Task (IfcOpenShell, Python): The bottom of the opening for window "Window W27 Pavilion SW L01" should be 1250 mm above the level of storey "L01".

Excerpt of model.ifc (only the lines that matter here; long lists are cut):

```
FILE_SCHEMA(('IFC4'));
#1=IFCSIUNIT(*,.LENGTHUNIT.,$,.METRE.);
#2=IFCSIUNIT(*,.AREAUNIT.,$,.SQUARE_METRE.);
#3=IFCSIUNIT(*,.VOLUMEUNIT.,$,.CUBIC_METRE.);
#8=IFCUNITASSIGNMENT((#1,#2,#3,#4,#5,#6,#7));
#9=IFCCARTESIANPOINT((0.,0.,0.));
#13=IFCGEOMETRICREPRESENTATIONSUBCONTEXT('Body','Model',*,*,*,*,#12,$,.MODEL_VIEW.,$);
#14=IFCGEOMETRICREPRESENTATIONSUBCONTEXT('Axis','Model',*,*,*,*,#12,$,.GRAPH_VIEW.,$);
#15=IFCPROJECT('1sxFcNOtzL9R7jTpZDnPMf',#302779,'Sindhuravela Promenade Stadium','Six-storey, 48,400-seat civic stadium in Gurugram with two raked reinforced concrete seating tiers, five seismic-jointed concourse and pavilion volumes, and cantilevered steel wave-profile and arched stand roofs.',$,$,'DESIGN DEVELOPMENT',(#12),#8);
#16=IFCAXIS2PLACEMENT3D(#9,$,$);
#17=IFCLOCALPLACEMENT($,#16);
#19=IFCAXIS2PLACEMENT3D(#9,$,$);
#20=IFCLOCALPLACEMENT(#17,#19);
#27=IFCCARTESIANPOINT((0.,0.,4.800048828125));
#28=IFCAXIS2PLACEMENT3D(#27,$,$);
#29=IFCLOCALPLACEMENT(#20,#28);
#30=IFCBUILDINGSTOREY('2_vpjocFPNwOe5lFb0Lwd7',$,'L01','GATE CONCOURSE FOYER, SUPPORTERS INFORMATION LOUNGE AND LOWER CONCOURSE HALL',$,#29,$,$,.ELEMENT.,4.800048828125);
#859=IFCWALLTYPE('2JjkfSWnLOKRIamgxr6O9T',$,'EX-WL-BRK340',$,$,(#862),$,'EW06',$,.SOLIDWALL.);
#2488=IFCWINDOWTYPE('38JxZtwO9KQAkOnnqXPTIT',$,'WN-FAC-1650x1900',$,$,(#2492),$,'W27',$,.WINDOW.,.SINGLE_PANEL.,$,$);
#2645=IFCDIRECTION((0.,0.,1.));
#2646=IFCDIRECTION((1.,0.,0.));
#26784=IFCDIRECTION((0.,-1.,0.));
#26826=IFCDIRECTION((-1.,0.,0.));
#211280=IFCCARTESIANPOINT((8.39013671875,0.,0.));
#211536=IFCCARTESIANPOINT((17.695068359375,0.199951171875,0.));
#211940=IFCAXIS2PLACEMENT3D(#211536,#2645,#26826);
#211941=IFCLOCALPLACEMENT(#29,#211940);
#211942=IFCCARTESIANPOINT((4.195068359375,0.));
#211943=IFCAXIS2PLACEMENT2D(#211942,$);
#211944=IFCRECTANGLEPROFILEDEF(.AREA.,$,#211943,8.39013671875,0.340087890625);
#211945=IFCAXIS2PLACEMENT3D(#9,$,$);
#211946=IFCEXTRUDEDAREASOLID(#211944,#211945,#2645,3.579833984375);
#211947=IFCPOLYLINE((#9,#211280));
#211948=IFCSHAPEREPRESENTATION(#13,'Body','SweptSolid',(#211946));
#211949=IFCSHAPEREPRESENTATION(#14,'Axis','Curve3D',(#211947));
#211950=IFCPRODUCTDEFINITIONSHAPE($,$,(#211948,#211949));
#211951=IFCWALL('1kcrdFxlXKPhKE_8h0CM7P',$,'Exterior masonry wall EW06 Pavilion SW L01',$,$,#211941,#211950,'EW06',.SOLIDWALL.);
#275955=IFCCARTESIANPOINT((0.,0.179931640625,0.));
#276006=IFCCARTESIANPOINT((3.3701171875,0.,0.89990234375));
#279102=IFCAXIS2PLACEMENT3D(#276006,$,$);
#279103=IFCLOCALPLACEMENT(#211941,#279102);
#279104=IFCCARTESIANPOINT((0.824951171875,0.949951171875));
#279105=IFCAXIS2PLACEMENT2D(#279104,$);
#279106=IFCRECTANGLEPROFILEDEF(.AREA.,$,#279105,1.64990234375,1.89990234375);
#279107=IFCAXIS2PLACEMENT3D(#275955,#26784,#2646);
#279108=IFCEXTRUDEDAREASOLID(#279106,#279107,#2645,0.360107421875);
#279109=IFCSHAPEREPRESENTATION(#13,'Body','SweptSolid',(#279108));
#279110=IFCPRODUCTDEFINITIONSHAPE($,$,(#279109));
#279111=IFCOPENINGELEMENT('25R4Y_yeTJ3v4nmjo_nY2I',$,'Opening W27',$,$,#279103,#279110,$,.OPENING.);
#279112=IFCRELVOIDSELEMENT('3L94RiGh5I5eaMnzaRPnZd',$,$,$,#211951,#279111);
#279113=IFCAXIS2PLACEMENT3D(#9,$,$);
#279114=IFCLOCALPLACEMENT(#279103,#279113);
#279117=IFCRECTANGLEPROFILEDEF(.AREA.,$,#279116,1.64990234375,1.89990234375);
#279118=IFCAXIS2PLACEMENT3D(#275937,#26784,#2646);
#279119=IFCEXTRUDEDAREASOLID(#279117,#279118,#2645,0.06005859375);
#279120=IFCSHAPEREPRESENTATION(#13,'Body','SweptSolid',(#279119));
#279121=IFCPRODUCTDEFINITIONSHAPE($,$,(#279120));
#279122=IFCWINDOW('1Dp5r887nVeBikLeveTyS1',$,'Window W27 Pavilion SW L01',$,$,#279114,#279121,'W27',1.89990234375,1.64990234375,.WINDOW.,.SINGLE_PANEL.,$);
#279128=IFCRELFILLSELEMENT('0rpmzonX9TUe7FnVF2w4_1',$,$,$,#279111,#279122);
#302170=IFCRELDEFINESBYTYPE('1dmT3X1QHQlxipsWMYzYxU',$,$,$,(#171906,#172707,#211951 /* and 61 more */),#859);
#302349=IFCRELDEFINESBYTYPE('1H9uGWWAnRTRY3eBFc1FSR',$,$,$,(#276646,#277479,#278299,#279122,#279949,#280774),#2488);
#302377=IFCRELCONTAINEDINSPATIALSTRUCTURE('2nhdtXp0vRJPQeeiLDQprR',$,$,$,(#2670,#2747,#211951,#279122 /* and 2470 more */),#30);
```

```python
import numpy as np
import ifcopenshell
import ifcopenshell.api.geometry
import ifcopenshell.geom
import ifcopenshell.util.element
import ifcopenshell.util.placement
import ifcopenshell.util.shape
import ifcopenshell.util.unit

model = ifcopenshell.open("model.ifc")
unit_scale = ifcopenshell.util.unit.calculate_unit_scale(model)

window = model.by_guid("1Dp5r887nVeBikLeveTyS1")
opening = window.FillsVoids[0].RelatingOpeningElement
storey = ifcopenshell.util.element.get_container(window, ifc_class="IfcBuildingStorey")
level = ifcopenshell.util.placement.get_local_placement(storey.ObjectPlacement)[2, 3]

# The opening's origin need not be at the sill, so measure its lowest point.
shape = ifcopenshell.geom.create_shape(ifcopenshell.geom.settings(), opening)
bottom = ifcopenshell.util.shape.get_shape_bottom_elevation(shape, shape.geometry) / unit_scale
dz = level + 1.25 / unit_scale - bottom

shift = np.array([0.0, 0.0, dz])
# The window is placed relative to its opening, so it follows when the opening moves.
matrix = ifcopenshell.util.placement.get_local_placement(opening.ObjectPlacement)
matrix[:3, 3] += shift
ifcopenshell.api.geometry.edit_object_placement(
    model, product=opening, matrix=matrix, is_si=False, should_transform_children=True
)

print(f"moved by {dz * unit_scale:+.3f} m")

model.write("model_updated.ifc")
```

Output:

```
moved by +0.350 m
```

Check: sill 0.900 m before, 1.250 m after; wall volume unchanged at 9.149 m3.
